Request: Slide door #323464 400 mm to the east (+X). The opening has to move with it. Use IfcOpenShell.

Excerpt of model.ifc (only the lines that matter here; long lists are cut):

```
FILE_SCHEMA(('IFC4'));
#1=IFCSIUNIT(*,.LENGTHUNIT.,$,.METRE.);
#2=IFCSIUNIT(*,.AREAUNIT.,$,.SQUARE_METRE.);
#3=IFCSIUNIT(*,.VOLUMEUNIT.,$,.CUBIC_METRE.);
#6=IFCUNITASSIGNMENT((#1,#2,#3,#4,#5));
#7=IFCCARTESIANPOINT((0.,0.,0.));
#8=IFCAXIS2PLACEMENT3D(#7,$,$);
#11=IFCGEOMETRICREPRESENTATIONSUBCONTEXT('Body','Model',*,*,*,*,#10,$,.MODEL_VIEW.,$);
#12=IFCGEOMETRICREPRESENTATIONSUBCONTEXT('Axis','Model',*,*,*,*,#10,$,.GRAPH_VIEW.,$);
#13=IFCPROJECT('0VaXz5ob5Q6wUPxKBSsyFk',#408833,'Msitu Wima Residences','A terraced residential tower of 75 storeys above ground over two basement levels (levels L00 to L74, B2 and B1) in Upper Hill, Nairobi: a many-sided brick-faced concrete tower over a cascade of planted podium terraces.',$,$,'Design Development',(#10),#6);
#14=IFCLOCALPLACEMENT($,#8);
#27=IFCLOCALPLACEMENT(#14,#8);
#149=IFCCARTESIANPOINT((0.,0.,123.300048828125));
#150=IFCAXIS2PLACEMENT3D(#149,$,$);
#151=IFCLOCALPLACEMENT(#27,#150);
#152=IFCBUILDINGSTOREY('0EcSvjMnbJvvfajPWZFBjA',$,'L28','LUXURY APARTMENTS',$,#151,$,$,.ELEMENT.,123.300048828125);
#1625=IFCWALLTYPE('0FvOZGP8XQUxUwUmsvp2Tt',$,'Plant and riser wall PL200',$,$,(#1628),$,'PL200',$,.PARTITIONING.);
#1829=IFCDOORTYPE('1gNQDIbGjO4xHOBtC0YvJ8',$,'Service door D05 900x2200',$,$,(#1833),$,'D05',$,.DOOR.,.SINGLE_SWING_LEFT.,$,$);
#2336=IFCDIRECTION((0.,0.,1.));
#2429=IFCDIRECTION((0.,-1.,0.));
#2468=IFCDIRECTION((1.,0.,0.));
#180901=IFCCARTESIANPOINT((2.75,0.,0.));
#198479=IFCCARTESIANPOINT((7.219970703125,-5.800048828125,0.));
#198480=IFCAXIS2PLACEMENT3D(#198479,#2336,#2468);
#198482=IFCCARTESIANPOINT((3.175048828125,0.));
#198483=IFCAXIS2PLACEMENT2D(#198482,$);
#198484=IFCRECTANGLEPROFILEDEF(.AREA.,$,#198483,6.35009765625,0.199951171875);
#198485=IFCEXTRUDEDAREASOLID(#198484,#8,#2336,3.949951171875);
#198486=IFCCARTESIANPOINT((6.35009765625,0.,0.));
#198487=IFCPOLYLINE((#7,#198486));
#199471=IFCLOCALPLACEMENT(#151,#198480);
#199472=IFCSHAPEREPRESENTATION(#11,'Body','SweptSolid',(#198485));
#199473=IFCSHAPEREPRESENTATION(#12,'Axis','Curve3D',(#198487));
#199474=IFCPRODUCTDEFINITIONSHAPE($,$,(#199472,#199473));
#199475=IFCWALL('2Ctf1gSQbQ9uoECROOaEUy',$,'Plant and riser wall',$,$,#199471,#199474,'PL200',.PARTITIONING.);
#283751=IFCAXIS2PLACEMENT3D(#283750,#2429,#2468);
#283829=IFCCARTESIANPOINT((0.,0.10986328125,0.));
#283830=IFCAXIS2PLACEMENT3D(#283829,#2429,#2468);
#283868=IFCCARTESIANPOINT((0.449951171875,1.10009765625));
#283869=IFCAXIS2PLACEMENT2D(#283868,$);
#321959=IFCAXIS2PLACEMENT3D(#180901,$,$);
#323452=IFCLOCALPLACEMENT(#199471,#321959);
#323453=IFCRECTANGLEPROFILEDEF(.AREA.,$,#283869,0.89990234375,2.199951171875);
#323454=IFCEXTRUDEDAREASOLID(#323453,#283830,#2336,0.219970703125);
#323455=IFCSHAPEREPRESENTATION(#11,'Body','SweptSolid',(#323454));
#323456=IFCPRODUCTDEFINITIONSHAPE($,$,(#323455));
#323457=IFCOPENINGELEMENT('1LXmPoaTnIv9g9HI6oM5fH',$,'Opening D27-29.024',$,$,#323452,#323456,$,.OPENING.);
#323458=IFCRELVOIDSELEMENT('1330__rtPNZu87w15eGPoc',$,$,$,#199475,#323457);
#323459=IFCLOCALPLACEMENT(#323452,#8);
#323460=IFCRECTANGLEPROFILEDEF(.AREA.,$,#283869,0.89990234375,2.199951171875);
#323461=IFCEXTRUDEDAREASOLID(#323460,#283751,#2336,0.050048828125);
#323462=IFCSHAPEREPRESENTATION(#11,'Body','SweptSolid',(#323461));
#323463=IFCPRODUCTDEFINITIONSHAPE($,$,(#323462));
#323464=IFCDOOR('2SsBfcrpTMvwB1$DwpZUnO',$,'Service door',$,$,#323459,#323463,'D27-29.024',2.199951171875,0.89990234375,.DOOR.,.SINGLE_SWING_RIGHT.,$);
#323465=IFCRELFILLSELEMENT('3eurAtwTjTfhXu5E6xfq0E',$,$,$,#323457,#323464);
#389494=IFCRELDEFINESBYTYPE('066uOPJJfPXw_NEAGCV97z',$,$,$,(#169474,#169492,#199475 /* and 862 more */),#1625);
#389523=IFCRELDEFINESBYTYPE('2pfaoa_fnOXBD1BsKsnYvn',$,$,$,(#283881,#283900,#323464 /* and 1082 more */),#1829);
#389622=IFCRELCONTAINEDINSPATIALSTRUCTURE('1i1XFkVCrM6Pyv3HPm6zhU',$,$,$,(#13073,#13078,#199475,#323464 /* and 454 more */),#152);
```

```python
import ifcopenshell
import ifcopenshell.api.geometry
import ifcopenshell.util.placement
import ifcopenshell.util.unit

model = ifcopenshell.open("model.ifc")
unit_scale = ifcopenshell.util.unit.calculate_unit_scale(model)

door = model.by_guid("2SsBfcrpTMvwB1$DwpZUnO")
opening = door.FillsVoids[0].RelatingOpeningElement
wall = opening.VoidsElements[0].RelatingBuildingElement

wall_matrix = ifcopenshell.util.placement.get_local_placement(wall.ObjectPlacement)
shift = wall_matrix[:3, 0] * 0.4 / unit_scale
before = ifcopenshell.util.placement.get_local_placement(door.ObjectPlacement)[:3, 3].copy()

# The door is placed relative to its opening, so it follows when the opening moves.
matrix = ifcopenshell.util.placement.get_local_placement(opening.ObjectPlacement)
matrix[:3, 3] += shift
ifcopenshell.api.geometry.edit_object_placement(
    model, product=opening, matrix=matrix, is_si=False, should_transform_children=True
)

after = ifcopenshell.util.placement.get_local_placement(door.ObjectPlacement)[:3, 3]
print("door moved by", (after - before).round(3) + 0.0)

model.write("model_updated.ifc")
```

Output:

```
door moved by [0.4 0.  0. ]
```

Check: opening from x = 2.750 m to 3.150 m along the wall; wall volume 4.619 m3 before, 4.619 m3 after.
